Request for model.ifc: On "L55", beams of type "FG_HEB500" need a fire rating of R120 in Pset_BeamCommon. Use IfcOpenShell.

First a look at what the model holds.

```python
import ifcopenshell
import ifcopenshell.util.element

model = ifcopenshell.open("model.ifc")
print(model.schema)
storey = next(s for s in model.by_type("IfcBuildingStorey") if s.Name == "L55")
beams = [e for e in ifcopenshell.util.element.get_decomposition(storey) if e.is_a("IfcBeam")]
seen = {}
for e in beams:
    element_type = ifcopenshell.util.element.get_type(e)
    key = (element_type.Name if element_type != e and element_type else None, ifcopenshell.util.element.get_pset(e, "Pset_BeamCommon", "FireRating"))
    seen[key] = seen.get(key, 0) + 1
for (name, value), count in sorted(seen.items(), key=str):
    print(count, "x", name, "|", value)
```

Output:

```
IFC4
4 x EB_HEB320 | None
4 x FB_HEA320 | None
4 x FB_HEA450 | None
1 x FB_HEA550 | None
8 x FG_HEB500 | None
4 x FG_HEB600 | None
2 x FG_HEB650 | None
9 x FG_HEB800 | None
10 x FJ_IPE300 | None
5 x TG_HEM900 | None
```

```python
import ifcopenshell
import ifcopenshell.api.pset
import ifcopenshell.util.element

model = ifcopenshell.open("model.ifc")

storey = next(s for s in model.by_type("IfcBuildingStorey") if s.Name == "L55")
beams = [e for e in ifcopenshell.util.element.get_decomposition(storey) if e.is_a("IfcBeam")]

count = 0
for e in beams:
    element_type = ifcopenshell.util.element.get_type(e)
    if element_type in (None, e) or element_type.Name != "FG_HEB500":
        continue
    # add_pset returns the element's existing set when there is one.
    pset = ifcopenshell.api.pset.add_pset(model, product=e, name="Pset_BeamCommon")
    ifcopenshell.api.pset.edit_pset(model, pset=pset, properties={"FireRating": "R120"})
    count += 1

print(count, "beams updated")

model.write("model_edited.ifc")
```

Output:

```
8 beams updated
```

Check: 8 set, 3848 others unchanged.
